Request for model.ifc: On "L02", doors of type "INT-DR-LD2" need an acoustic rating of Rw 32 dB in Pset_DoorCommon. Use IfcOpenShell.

First a look at what the model holds.

```python
import ifcopenshell
import ifcopenshell.util.element

model = ifcopenshell.open("model.ifc")
print(model.schema)
storey = next(s for s in model.by_type("IfcBuildingStorey") if s.Name == "L02")
doors = [e for e in ifcopenshell.util.element.get_decomposition(storey) if e.is_a("IfcDoor")]
seen = {}
for e in doors:
    element_type = ifcopenshell.util.element.get_type(e)
    key = (element_type.Name if element_type != e and element_type else None, ifcopenshell.util.element.get_pset(e, "Pset_DoorCommon", "AcousticRating"))
    seen[key] = seen.get(key, 0) + 1
for (name, value), count in sorted(seen.items(), key=str):
    print(count, "x", name, "|", value)
```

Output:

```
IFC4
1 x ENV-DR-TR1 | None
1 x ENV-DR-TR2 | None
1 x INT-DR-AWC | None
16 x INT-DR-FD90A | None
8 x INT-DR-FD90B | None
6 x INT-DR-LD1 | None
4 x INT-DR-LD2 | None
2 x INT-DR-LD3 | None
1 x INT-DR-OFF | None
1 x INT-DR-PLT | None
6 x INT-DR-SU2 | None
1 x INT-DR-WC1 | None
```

```python
import ifcopenshell
import ifcopenshell.api.pset
import ifcopenshell.util.element

model = ifcopenshell.open("model.ifc")

storey = next(s for s in model.by_type("IfcBuildingStorey") if s.Name == "L02")
doors = [e for e in ifcopenshell.util.element.get_decomposition(storey) if e.is_a("IfcDoor")]

count = 0
for e in doors:
    element_type = ifcopenshell.util.element.get_type(e)
    if element_type in (None, e) or element_type.Name != "INT-DR-LD2":
        continue
    # add_pset returns the element's existing set when there is one.
    pset = ifcopenshell.api.pset.add_pset(model, product=e, name="Pset_DoorCommon")
    ifcopenshell.api.pset.edit_pset(model, pset=pset, properties={"AcousticRating": "Rw 32 dB"})
    count += 1

print(count, "doors updated")

model.write("model-out.ifc")
```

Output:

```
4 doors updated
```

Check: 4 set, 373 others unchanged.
